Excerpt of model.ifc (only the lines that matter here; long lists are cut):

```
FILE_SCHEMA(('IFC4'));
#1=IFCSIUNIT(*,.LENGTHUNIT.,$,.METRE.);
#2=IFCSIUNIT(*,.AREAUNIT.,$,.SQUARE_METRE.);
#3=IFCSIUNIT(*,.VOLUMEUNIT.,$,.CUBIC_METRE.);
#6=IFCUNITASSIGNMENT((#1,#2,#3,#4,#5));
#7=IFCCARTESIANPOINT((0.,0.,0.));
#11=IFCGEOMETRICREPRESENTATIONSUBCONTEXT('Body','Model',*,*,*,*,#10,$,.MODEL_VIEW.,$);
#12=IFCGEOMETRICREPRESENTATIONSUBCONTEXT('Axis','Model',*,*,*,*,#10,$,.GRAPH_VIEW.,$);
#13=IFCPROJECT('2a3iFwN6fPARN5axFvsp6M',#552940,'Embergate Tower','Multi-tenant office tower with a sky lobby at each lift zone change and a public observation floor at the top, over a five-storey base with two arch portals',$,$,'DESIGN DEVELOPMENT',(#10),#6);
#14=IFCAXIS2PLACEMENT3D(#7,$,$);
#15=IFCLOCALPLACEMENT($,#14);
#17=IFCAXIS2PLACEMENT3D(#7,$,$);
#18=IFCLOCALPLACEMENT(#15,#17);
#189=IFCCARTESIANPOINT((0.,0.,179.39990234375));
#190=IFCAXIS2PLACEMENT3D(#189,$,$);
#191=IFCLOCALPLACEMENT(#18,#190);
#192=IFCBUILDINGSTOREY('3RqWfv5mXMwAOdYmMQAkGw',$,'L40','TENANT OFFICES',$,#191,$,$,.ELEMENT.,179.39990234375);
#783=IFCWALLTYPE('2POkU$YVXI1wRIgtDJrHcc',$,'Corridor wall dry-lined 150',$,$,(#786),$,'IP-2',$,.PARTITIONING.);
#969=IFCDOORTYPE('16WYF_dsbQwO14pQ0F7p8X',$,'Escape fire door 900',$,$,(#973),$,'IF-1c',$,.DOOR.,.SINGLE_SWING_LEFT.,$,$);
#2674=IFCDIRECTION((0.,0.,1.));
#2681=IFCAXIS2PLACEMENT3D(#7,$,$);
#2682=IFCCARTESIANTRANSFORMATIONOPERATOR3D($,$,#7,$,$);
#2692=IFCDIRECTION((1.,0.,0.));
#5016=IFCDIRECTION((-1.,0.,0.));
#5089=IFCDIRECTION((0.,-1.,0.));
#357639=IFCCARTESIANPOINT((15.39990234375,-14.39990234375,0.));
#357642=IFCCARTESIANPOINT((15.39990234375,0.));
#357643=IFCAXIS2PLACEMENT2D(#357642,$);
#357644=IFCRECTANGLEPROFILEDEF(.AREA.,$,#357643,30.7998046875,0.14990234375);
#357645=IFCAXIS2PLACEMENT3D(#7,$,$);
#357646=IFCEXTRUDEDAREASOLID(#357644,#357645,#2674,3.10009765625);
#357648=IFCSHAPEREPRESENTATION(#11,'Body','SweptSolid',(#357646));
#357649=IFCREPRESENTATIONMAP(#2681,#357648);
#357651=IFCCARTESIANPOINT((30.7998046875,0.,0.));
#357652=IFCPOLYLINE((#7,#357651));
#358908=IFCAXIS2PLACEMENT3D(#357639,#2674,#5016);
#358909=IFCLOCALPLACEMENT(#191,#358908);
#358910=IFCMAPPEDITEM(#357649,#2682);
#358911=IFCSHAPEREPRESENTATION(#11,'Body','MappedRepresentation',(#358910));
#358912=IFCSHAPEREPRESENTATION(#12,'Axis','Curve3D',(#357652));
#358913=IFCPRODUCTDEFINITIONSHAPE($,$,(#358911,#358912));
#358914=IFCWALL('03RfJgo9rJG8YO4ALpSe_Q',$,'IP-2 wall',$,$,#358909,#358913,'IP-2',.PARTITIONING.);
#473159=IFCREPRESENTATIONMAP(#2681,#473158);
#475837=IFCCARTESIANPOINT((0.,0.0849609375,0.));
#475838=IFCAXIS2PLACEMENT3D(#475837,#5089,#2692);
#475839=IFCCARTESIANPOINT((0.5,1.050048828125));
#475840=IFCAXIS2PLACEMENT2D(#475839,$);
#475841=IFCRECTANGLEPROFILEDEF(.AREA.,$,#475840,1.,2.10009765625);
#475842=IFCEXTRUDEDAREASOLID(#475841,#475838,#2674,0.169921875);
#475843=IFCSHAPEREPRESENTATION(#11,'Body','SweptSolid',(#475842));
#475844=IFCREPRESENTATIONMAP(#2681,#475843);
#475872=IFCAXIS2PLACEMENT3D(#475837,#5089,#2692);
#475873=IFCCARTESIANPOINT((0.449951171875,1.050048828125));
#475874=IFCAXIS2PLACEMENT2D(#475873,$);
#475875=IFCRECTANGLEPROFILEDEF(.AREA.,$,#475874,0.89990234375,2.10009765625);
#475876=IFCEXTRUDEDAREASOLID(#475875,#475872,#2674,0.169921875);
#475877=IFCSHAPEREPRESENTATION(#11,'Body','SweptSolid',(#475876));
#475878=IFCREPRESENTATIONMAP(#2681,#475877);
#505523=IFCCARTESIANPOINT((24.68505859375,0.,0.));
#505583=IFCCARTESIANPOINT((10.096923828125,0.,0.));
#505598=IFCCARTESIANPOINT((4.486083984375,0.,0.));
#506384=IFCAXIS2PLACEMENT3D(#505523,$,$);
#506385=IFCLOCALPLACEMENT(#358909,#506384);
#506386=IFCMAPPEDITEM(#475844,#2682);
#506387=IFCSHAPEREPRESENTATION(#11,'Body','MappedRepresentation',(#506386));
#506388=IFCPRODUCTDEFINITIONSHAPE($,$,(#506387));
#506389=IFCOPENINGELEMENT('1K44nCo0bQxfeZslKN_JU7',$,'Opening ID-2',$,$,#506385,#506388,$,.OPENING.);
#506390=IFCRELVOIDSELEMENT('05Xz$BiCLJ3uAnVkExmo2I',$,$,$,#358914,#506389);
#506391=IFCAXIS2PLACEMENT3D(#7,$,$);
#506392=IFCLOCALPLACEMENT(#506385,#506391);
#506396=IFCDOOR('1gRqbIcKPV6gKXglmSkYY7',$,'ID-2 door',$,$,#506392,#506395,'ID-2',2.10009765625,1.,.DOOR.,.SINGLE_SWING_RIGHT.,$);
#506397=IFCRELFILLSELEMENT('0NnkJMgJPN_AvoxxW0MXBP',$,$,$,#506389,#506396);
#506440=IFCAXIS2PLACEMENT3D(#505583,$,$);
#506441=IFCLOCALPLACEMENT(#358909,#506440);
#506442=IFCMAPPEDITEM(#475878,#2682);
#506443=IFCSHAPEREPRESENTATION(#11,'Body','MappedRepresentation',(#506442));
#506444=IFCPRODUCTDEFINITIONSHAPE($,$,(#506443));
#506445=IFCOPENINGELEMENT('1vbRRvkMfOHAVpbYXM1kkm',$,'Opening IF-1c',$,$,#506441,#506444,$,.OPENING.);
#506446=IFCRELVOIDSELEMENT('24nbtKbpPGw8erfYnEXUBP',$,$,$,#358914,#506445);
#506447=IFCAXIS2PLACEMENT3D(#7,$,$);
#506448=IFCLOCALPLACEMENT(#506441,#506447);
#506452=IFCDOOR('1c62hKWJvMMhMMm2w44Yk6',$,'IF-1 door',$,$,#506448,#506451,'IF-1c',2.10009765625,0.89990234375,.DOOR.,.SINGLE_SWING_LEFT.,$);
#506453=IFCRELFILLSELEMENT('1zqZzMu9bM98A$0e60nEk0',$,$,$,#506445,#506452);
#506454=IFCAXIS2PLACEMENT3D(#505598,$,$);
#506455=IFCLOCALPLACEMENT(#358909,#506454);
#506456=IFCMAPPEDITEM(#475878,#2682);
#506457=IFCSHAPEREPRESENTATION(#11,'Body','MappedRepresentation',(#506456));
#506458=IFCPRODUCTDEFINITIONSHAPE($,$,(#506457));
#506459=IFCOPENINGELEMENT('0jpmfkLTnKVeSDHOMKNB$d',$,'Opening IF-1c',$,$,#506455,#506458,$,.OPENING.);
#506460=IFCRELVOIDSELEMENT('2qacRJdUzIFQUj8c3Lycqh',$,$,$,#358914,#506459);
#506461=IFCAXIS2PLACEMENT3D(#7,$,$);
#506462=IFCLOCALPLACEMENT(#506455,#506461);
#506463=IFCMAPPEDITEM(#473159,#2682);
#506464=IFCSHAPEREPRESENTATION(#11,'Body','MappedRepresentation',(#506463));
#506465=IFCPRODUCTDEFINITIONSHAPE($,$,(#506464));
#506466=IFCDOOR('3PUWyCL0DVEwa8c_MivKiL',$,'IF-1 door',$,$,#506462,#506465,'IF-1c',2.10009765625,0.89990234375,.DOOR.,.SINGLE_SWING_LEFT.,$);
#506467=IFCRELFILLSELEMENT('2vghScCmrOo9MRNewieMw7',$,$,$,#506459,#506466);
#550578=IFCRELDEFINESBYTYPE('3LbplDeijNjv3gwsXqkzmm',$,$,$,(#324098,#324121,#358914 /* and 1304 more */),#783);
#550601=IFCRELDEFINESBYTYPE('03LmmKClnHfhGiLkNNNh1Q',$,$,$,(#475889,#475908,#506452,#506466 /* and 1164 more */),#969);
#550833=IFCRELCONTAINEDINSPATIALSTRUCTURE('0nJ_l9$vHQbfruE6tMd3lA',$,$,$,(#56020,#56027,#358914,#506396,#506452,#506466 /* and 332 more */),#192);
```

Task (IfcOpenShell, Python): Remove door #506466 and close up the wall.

```python
import ifcopenshell
import ifcopenshell.api.feature
import ifcopenshell.api.root
import ifcopenshell.geom
import ifcopenshell.util.shape

model = ifcopenshell.open("model.ifc")
settings = ifcopenshell.geom.settings()


def volume(element):
    """Net volume in cubic metres, openings subtracted."""
    shape = ifcopenshell.geom.create_shape(settings, element)
    return ifcopenshell.util.shape.get_volume(shape.geometry)


door = model.by_guid("3PUWyCL0DVEwa8c_MivKiL")
opening = door.FillsVoids[0].RelatingOpeningElement
wall = opening.VoidsElements[0].RelatingBuildingElement
before = volume(wall)

ifcopenshell.api.root.remove_product(model, product=door)
ifcopenshell.api.feature.remove_feature(model, feature=opening)

after = volume(wall)

print(f"wall volume {before:.3f} -> {after:.3f} m3")

model.write("model_rev.ifc")
```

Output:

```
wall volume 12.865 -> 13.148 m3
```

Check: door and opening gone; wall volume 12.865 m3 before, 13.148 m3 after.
